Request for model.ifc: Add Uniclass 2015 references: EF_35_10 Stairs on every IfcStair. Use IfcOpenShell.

First a look at what the model holds.

```python
import ifcopenshell

model = ifcopenshell.open("model.ifc")
print(model.schema)
print("classifications:", [c.Name for c in model.by_type("IfcClassification")])
for ifc_class in ("IfcDoor", "IfcRoof", "IfcStair", "IfcWall", "IfcWindow"):
    print(ifc_class, len(model.by_type(ifc_class)))
```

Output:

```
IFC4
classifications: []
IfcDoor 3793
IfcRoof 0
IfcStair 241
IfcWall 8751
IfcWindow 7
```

```python
import ifcopenshell
import ifcopenshell.api.classification

model = ifcopenshell.open("model.ifc")

system = ifcopenshell.api.classification.add_classification(model, classification="Uniclass 2015")

codes = {
    "IfcStair": ("EF_35_10", "Stairs"),
}
for ifc_class, (code, name) in codes.items():
    products = model.by_type(ifc_class)
    ifcopenshell.api.classification.add_reference(
        model, products=products, classification=system, identification=code, name=name
    )
    print(code, len(products))

model.write("model_rev.ifc")
```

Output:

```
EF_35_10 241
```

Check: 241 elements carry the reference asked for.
